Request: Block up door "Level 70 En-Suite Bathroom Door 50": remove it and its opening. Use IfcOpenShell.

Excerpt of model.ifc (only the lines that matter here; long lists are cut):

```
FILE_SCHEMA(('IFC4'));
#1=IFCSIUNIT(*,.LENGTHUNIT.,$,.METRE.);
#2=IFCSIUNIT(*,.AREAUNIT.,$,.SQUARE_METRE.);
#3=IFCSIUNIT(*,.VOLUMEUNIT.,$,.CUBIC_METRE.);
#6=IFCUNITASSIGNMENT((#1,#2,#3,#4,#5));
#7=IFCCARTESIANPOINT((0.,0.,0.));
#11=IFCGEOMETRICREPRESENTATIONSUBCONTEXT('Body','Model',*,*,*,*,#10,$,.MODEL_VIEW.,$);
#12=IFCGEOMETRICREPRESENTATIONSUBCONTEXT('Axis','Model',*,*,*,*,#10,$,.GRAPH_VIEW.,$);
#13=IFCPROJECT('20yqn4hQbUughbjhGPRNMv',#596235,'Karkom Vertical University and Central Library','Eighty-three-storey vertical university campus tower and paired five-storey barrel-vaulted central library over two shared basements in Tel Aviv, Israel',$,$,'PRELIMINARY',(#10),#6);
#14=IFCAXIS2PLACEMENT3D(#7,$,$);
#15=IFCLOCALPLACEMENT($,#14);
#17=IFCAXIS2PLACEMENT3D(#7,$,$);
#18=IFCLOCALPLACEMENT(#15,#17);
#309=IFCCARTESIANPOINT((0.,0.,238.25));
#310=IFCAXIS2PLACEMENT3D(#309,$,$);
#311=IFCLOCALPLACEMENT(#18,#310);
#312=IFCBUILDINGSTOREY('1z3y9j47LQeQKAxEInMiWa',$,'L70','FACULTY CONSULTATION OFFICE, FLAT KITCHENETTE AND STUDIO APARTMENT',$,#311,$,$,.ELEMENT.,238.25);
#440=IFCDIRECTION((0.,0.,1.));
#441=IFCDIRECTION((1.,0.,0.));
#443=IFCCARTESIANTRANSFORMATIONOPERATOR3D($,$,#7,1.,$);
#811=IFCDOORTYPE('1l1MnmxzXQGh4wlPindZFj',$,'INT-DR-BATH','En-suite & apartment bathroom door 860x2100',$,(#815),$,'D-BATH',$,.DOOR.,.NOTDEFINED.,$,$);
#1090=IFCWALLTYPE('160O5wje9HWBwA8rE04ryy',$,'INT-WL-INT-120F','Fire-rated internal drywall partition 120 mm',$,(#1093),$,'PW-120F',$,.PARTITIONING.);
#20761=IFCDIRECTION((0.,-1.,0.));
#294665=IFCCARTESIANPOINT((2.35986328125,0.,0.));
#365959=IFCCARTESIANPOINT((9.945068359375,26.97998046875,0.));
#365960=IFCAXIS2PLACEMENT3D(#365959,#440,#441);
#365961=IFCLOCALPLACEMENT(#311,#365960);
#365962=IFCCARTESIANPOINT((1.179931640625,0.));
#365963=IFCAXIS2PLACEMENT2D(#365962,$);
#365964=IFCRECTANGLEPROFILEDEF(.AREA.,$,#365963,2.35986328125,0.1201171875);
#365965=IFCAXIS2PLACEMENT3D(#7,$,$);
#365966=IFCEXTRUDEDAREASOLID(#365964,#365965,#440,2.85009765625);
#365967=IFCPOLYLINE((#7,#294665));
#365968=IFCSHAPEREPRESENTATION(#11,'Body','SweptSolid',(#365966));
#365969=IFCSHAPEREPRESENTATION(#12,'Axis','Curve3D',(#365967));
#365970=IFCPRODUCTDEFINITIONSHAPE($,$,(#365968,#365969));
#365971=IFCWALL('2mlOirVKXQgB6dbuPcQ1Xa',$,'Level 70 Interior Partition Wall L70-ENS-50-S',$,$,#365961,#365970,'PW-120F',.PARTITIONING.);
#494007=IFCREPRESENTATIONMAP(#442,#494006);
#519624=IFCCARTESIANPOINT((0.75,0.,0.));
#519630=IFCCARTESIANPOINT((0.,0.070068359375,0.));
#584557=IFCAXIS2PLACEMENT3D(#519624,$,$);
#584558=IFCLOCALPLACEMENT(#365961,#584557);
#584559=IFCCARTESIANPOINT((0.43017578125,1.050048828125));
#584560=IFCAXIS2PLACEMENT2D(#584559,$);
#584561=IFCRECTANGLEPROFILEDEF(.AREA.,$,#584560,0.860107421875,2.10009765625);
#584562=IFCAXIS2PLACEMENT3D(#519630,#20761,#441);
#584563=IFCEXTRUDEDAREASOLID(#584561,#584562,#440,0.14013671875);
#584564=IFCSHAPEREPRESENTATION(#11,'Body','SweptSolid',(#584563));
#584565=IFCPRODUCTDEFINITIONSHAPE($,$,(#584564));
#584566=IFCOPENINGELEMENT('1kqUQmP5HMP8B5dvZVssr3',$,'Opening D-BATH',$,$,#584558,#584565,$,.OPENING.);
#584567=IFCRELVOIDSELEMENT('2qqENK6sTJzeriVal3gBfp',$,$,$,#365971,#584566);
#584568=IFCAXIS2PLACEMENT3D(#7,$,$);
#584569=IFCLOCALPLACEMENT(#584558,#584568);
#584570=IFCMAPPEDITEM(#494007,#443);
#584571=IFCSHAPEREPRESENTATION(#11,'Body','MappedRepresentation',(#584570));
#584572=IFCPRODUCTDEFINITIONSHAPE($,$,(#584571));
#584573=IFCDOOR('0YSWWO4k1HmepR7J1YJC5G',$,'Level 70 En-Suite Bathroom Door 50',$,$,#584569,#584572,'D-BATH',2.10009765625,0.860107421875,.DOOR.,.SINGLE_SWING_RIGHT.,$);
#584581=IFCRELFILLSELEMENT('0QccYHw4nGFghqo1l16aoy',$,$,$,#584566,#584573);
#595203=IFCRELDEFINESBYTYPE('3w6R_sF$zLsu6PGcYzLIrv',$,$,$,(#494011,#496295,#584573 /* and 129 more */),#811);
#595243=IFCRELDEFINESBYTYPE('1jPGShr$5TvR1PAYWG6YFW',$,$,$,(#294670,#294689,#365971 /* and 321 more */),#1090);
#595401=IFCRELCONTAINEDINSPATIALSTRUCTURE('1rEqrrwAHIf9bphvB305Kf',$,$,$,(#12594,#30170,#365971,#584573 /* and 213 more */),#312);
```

```python
import ifcopenshell
import ifcopenshell.api.feature
import ifcopenshell.api.root
import ifcopenshell.geom
import ifcopenshell.util.shape

model = ifcopenshell.open("model.ifc")
settings = ifcopenshell.geom.settings()


def volume(element):
    """Net volume in cubic metres, openings subtracted."""
    shape = ifcopenshell.geom.create_shape(settings, element)
    return ifcopenshell.util.shape.get_volume(shape.geometry)


door = model.by_guid("0YSWWO4k1HmepR7J1YJC5G")
opening = door.FillsVoids[0].RelatingOpeningElement
wall = opening.VoidsElements[0].RelatingBuildingElement
before = volume(wall)

ifcopenshell.api.root.remove_product(model, product=door)
ifcopenshell.api.feature.remove_feature(model, feature=opening)

after = volume(wall)

print(f"wall volume {before:.3f} -> {after:.3f} m3")

model.write("model-out.ifc")
```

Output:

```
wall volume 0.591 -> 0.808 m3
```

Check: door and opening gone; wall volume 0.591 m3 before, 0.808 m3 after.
